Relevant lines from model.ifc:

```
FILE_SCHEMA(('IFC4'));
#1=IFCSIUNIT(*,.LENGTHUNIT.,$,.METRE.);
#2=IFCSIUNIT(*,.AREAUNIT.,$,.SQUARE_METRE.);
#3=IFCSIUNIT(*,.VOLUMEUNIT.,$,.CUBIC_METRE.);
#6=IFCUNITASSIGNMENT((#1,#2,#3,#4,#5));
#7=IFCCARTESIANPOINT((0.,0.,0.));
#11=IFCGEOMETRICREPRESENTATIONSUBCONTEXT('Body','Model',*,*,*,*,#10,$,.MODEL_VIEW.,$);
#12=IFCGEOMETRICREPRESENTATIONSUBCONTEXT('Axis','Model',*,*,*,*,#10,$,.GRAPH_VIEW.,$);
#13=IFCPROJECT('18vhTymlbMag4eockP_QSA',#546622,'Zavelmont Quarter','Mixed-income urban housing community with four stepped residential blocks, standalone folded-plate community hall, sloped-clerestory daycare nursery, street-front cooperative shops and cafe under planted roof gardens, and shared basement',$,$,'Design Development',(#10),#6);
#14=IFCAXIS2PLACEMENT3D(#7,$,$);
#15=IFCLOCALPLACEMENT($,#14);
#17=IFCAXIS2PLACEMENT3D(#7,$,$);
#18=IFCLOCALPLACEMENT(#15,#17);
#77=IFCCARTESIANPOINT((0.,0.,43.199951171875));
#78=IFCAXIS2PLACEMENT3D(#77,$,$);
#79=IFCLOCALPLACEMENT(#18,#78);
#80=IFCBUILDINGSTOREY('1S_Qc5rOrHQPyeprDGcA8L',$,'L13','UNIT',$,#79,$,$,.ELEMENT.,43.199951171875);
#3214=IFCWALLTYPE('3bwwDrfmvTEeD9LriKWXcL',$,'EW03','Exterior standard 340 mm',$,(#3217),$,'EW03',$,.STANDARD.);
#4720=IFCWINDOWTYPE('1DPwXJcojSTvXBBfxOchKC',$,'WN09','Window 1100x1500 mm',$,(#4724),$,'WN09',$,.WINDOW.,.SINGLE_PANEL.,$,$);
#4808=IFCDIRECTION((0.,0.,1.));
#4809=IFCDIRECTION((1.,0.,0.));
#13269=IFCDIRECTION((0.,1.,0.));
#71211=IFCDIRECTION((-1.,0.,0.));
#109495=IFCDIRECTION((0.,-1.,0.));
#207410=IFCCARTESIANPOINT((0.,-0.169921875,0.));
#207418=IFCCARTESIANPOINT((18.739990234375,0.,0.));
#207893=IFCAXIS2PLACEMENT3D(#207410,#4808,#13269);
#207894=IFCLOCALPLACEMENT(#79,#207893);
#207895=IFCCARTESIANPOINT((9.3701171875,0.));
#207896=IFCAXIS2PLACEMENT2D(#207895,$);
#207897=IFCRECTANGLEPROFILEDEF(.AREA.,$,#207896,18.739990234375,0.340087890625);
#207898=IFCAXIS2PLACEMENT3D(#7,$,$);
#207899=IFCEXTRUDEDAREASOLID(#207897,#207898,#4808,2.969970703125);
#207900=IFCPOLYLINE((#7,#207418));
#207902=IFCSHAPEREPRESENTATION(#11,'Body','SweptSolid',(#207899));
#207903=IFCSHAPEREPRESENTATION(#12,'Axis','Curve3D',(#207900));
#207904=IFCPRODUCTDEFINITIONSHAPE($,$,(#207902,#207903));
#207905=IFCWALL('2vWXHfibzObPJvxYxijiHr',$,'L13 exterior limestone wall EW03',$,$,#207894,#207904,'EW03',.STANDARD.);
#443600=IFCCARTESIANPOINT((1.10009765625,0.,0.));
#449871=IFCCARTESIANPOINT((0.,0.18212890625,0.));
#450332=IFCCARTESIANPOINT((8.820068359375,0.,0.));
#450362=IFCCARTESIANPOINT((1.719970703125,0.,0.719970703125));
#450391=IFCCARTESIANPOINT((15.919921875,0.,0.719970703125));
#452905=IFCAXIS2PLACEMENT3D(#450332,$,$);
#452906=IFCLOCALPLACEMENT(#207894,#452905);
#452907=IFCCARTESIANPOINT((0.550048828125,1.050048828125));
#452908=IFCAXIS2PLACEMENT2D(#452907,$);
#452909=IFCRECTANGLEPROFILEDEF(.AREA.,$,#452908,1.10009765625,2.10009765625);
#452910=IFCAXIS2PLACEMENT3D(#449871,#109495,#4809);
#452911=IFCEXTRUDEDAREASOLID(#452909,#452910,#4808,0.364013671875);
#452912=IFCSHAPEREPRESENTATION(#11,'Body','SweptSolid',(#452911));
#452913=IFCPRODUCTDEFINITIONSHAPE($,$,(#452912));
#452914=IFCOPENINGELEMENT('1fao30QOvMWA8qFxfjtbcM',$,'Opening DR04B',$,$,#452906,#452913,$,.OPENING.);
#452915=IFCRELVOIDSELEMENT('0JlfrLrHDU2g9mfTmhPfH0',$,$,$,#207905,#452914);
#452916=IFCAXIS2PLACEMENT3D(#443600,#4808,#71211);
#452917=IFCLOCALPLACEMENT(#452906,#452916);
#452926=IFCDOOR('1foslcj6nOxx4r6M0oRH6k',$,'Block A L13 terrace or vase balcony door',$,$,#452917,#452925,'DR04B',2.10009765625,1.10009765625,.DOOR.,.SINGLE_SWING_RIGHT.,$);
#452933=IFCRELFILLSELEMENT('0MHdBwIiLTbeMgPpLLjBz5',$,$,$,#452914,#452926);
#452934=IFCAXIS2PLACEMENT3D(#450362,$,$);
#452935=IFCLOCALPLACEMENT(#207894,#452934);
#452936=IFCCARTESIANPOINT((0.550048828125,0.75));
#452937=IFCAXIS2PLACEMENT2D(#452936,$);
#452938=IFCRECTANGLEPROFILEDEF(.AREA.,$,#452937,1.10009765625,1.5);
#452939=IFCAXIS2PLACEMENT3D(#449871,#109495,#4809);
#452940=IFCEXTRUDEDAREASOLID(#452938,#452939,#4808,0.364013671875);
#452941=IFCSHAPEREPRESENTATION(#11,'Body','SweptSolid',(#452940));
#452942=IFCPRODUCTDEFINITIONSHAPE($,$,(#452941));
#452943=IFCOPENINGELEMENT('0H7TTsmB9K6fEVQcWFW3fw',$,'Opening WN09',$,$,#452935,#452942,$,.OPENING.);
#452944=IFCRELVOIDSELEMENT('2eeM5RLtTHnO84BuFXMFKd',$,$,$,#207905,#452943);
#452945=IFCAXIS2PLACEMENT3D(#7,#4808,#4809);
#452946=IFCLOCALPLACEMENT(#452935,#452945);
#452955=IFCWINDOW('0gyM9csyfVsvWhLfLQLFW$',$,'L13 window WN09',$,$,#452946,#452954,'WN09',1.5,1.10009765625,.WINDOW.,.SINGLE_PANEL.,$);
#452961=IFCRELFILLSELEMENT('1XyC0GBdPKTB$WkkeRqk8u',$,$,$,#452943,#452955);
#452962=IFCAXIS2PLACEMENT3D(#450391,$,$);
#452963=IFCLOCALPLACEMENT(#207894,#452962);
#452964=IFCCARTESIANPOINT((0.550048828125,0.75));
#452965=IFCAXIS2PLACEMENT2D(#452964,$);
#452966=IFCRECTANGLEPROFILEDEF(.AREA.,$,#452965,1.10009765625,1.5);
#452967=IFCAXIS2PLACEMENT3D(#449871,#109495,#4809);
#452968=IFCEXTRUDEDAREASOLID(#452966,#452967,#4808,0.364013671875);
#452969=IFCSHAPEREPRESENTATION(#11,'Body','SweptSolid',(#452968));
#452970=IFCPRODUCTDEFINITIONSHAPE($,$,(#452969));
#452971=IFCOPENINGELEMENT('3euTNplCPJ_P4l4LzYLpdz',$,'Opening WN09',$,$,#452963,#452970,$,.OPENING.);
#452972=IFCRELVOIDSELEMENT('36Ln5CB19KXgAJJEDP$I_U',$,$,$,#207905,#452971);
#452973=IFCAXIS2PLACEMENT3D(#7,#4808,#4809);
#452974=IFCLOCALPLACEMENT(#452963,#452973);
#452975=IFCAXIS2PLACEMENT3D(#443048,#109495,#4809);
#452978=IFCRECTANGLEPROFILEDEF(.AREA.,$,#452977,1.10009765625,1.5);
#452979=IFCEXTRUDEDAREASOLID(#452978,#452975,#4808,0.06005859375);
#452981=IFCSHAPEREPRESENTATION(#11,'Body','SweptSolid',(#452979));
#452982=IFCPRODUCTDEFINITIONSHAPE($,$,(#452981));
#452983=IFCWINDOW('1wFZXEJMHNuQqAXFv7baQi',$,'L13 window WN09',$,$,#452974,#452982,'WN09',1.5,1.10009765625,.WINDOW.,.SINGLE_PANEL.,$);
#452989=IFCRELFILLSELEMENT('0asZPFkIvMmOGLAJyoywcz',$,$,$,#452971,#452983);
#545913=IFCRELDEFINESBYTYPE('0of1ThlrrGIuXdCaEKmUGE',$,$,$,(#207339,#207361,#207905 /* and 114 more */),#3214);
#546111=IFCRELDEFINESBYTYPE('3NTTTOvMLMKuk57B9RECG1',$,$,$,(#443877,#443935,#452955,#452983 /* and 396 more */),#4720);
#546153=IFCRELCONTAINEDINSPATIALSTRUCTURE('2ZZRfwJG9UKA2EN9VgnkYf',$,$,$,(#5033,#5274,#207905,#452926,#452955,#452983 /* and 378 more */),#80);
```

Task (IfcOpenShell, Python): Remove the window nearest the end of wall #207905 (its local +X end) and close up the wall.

```python
import ifcopenshell
import ifcopenshell.api.feature
import ifcopenshell.api.root
import ifcopenshell.geom
import ifcopenshell.util.shape

model = ifcopenshell.open("model.ifc")
settings = ifcopenshell.geom.settings()


def volume(element):
    """Net volume in cubic metres, openings subtracted."""
    shape = ifcopenshell.geom.create_shape(settings, element)
    return ifcopenshell.util.shape.get_volume(shape.geometry)


window = model.by_guid("1wFZXEJMHNuQqAXFv7baQi")
opening = window.FillsVoids[0].RelatingOpeningElement
wall = opening.VoidsElements[0].RelatingBuildingElement
before = volume(wall)

ifcopenshell.api.root.remove_product(model, product=window)
ifcopenshell.api.feature.remove_feature(model, feature=opening)

after = volume(wall)

print(f"wall volume {before:.3f} -> {after:.3f} m3")

model.write("model_v2.ifc")
```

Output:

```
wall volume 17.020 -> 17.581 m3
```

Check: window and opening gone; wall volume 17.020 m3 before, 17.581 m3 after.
